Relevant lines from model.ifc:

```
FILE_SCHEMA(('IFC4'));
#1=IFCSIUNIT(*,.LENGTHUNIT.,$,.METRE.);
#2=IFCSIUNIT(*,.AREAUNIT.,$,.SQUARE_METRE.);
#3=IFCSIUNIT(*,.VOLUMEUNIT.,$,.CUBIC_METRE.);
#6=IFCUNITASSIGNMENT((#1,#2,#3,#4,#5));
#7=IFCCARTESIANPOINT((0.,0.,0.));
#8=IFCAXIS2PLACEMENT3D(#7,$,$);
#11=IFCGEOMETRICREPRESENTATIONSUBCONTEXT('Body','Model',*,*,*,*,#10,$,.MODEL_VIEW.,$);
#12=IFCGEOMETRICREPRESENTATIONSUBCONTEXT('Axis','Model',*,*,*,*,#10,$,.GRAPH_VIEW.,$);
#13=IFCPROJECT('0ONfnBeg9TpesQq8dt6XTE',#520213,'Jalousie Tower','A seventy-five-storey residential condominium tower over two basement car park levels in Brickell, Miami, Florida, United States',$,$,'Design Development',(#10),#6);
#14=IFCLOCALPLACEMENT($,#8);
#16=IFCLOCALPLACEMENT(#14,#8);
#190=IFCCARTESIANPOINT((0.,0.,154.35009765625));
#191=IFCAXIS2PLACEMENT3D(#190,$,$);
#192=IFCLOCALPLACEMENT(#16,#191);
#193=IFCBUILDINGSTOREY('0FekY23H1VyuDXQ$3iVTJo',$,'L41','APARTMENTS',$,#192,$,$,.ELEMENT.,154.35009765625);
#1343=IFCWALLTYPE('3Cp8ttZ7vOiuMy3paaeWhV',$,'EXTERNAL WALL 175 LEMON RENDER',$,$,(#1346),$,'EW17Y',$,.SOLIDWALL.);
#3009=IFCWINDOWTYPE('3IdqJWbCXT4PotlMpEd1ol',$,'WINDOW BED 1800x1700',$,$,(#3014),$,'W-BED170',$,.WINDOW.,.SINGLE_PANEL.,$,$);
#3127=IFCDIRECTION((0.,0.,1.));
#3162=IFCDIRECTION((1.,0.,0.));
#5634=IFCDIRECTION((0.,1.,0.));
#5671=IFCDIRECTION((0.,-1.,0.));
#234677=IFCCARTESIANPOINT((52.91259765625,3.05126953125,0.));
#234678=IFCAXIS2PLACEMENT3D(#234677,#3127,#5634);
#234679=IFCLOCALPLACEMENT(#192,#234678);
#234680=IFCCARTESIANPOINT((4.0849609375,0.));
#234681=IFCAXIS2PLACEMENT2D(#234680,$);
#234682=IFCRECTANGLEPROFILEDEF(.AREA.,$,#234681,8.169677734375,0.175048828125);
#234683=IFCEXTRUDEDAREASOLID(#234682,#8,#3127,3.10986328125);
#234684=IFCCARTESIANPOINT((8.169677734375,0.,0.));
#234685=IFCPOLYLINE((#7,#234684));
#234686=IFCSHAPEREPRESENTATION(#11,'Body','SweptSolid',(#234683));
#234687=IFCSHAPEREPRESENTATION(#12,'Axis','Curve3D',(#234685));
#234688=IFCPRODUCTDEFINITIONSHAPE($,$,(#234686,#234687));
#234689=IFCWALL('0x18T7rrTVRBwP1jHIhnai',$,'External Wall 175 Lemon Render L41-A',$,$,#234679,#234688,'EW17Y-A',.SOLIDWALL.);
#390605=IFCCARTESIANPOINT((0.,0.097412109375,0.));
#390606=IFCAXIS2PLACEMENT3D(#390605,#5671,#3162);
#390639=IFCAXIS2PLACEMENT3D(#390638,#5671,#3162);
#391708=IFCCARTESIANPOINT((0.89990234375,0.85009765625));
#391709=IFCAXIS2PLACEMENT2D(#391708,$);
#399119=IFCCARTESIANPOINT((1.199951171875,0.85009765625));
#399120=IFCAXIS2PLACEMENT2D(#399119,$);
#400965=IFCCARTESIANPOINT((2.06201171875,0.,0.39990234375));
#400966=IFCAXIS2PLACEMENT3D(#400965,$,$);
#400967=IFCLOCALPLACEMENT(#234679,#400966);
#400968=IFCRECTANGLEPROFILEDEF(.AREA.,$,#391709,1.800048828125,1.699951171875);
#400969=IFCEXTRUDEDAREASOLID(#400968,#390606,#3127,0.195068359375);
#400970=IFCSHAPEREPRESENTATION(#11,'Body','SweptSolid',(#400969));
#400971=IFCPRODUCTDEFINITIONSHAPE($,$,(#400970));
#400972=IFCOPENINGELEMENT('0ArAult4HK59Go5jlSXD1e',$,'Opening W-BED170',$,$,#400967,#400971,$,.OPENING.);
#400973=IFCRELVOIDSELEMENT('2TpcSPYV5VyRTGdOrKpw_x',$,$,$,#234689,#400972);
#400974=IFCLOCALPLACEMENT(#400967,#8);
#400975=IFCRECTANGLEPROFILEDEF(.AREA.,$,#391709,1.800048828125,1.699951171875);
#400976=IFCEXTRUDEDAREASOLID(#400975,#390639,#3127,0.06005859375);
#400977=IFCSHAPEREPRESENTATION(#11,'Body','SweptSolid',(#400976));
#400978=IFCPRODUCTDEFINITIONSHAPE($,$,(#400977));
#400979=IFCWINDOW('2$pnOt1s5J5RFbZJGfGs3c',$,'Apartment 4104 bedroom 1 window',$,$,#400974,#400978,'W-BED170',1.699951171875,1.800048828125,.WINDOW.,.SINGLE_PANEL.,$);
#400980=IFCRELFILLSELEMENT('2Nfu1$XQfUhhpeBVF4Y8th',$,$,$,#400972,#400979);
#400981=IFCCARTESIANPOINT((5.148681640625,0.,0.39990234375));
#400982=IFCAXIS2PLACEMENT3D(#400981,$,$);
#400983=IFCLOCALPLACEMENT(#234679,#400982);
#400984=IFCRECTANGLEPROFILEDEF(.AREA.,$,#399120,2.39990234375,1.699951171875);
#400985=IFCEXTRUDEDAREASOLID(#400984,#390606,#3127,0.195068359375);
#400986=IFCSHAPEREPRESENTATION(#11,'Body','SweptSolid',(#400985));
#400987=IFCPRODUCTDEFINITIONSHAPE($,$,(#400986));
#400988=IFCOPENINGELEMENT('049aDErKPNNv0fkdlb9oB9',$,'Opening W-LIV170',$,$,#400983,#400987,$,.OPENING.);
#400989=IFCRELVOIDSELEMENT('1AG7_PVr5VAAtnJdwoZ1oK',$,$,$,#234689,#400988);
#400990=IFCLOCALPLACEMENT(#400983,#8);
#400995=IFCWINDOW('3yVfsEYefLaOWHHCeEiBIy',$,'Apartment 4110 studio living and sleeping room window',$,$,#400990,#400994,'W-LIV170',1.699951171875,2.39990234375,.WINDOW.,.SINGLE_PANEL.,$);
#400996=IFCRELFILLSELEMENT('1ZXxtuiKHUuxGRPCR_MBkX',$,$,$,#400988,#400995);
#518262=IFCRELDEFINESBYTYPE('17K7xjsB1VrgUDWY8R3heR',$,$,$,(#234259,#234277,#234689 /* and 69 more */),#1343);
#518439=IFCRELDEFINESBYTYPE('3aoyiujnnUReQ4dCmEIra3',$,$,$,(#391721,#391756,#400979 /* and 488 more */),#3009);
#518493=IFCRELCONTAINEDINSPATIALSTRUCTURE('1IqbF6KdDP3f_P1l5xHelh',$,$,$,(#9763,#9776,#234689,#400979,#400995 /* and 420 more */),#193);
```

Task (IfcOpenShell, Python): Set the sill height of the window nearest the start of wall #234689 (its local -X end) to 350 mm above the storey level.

```python
import numpy as np
import ifcopenshell
import ifcopenshell.api.geometry
import ifcopenshell.geom
import ifcopenshell.util.element
import ifcopenshell.util.placement
import ifcopenshell.util.shape
import ifcopenshell.util.unit

model = ifcopenshell.open("model.ifc")
unit_scale = ifcopenshell.util.unit.calculate_unit_scale(model)

window = model.by_guid("2$pnOt1s5J5RFbZJGfGs3c")
opening = window.FillsVoids[0].RelatingOpeningElement
storey = ifcopenshell.util.element.get_container(window, ifc_class="IfcBuildingStorey")
level = ifcopenshell.util.placement.get_local_placement(storey.ObjectPlacement)[2, 3]

# The opening's origin need not be at the sill, so measure its lowest point.
shape = ifcopenshell.geom.create_shape(ifcopenshell.geom.settings(), opening)
bottom = ifcopenshell.util.shape.get_shape_bottom_elevation(shape, shape.geometry) / unit_scale
dz = level + 0.35 / unit_scale - bottom

shift = np.array([0.0, 0.0, dz])
# The window is placed relative to its opening, so it follows when the opening moves.
matrix = ifcopenshell.util.placement.get_local_placement(opening.ObjectPlacement)
matrix[:3, 3] += shift
ifcopenshell.api.geometry.edit_object_placement(
    model, product=opening, matrix=matrix, is_si=False, should_transform_children=True
)

print(f"moved by {dz * unit_scale:+.3f} m")

model.write("model_v2.ifc")
```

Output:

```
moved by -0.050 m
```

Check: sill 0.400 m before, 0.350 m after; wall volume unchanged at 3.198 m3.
